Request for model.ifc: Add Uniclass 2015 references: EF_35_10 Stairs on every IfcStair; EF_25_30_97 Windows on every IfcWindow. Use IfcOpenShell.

First a look at what the model holds.

```python
import ifcopenshell

model = ifcopenshell.open("model.ifc")
print(model.schema)
print("classifications:", [c.Name for c in model.by_type("IfcClassification")])
for ifc_class in ("IfcDoor", "IfcRoof", "IfcStair", "IfcWall", "IfcWindow"):
    print(ifc_class, len(model.by_type(ifc_class)))
```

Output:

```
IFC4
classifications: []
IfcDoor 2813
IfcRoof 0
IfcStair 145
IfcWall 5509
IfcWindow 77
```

```python
import ifcopenshell
import ifcopenshell.api.classification

model = ifcopenshell.open("model.ifc")

system = ifcopenshell.api.classification.add_classification(model, classification="Uniclass 2015")

codes = {
    "IfcStair": ("EF_35_10", "Stairs"),
    "IfcWindow": ("EF_25_30_97", "Windows"),
}
for ifc_class, (code, name) in codes.items():
    products = model.by_type(ifc_class)
    ifcopenshell.api.classification.add_reference(
        model, products=products, classification=system, identification=code, name=name
    )
    print(code, len(products))

model.write("model-out.ifc")
```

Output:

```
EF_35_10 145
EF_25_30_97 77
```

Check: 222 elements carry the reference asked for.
